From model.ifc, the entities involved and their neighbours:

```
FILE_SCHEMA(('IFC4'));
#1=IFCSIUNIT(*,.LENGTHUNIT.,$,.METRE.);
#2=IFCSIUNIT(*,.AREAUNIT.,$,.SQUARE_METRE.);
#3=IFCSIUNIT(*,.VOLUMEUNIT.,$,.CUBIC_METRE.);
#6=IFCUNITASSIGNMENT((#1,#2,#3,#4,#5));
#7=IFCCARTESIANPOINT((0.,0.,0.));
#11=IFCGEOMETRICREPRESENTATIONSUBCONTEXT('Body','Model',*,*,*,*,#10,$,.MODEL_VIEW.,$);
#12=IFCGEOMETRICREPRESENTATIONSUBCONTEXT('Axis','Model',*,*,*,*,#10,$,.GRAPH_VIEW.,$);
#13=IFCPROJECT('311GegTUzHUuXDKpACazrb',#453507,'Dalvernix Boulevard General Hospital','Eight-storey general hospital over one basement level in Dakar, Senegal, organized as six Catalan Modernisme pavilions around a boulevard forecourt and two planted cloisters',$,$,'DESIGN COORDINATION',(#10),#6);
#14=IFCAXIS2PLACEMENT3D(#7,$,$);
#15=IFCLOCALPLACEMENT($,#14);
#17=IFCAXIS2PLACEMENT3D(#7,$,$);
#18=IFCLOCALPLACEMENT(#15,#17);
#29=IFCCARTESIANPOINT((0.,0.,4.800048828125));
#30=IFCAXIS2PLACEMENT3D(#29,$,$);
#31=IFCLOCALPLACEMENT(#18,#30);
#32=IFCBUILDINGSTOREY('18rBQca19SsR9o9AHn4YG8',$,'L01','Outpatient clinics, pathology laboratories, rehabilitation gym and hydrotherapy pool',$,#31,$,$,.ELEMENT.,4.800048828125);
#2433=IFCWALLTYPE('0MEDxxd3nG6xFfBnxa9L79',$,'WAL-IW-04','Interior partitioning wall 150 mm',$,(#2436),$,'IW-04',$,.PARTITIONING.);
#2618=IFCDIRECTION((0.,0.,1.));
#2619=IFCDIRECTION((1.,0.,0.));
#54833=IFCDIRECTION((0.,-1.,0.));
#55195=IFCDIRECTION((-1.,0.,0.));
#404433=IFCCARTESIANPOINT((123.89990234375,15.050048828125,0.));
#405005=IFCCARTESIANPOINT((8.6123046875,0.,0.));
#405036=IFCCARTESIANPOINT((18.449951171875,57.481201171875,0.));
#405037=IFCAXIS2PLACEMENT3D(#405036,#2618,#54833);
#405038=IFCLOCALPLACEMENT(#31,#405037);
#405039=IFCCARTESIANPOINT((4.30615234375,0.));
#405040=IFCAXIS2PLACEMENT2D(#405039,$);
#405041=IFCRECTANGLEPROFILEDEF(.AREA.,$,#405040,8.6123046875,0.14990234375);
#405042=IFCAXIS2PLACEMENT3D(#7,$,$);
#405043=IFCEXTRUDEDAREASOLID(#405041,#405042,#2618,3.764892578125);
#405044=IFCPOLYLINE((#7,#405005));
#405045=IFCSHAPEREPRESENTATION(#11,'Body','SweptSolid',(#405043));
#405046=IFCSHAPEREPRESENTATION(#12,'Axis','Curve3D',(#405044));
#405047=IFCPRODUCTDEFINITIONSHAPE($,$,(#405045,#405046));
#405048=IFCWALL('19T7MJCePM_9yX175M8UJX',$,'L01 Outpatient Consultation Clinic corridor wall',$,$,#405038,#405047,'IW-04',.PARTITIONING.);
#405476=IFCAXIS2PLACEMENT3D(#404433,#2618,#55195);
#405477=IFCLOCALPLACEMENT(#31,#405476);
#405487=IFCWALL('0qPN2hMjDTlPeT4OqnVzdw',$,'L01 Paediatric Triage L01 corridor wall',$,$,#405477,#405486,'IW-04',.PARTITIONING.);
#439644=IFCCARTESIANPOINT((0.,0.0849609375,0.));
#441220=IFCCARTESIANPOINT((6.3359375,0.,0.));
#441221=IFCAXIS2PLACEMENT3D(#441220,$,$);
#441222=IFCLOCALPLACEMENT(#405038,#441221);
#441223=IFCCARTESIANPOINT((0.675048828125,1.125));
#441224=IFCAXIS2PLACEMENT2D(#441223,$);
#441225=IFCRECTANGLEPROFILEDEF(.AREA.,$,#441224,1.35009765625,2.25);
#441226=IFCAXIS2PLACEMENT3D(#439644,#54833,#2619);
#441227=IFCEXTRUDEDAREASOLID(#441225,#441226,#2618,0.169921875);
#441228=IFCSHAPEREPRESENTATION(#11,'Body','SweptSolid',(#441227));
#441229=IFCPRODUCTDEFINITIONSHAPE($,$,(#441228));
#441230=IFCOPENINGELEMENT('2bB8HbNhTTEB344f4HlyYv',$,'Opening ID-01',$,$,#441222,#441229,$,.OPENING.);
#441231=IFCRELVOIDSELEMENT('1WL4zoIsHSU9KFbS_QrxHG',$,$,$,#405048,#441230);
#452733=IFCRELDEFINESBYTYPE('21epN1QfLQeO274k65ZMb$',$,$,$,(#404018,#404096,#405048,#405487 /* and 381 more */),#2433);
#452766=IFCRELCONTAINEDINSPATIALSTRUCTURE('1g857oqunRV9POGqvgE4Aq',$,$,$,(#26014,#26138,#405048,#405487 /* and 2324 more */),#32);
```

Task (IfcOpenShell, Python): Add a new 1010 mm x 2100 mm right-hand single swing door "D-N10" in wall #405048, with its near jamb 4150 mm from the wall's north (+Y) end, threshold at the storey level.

```python
import numpy as np
import ifcopenshell
import ifcopenshell.api.feature
import ifcopenshell.api.geometry
import ifcopenshell.api.root
import ifcopenshell.api.spatial
import ifcopenshell.geom
import ifcopenshell.util.element
import ifcopenshell.util.placement
import ifcopenshell.util.representation
import ifcopenshell.util.shape
import ifcopenshell.util.unit

model = ifcopenshell.open("model.ifc")
unit_scale = ifcopenshell.util.unit.calculate_unit_scale(model)
settings = ifcopenshell.geom.settings()


def volume(element):
    """Net volume in cubic metres, openings subtracted."""
    shape = ifcopenshell.geom.create_shape(settings, element)
    return ifcopenshell.util.shape.get_volume(shape.geometry)


wall = model.by_id(405048)
storey = ifcopenshell.util.element.get_container(wall, ifc_class="IfcBuildingStorey")
context = ifcopenshell.util.representation.get_context(model, "Model", "Body", "MODEL_VIEW")
before = volume(wall)

width, height, from_end, sill = 1.01, 2.1, 4.15, 0.0  # metres

# The wall runs along its own X axis, and the end named is its -X end.
wall_shape = ifcopenshell.geom.create_shape(settings, wall)
x, y, z = ifcopenshell.util.shape.get_vertices(wall_shape.geometry).T
start = x.min() + from_end
face, thickness = float(y.min()), float(y.max() - y.min())
wall_matrix = ifcopenshell.util.placement.get_local_placement(wall.ObjectPlacement)
level = ifcopenshell.util.placement.get_local_placement(storey.ObjectPlacement)[2, 3]


def in_wall(x, y):
    """Placement at x, y metres in the wall's axes, at sill height."""
    matrix = wall_matrix.copy()
    matrix[:, 3] = wall_matrix @ np.array([x / unit_scale, y / unit_scale, 0.0, 1.0])
    matrix[2, 3] = level + sill / unit_scale
    return matrix


# Opening: a box that overshoots both wall faces by 50 mm.
opening = ifcopenshell.api.root.create_entity(model, ifc_class="IfcOpeningElement", predefined_type="OPENING")
box = ifcopenshell.api.geometry.add_wall_representation(
    model, context=context, length=width, height=height, thickness=thickness + 0.1
)
ifcopenshell.api.geometry.assign_representation(model, product=opening, representation=box)
ifcopenshell.api.geometry.edit_object_placement(model, product=opening, matrix=in_wall(start, face - 0.05), is_si=False)
ifcopenshell.api.feature.add_feature(model, feature=opening, element=wall)

door = ifcopenshell.api.root.create_entity(model, ifc_class="IfcDoor", name="D-N10", predefined_type="DOOR")
door.OverallWidth, door.OverallHeight = width / unit_scale, height / unit_scale
door.OperationType = "SINGLE_SWING_RIGHT"
body = ifcopenshell.api.geometry.add_door_representation(
    model,
    context=context,
    overall_width=door.OverallWidth,
    overall_height=door.OverallHeight,
    operation_type="SINGLE_SWING_RIGHT",
    lining_properties={"LiningDepth": thickness / unit_scale, "ThresholdDepth": thickness / unit_scale},
)
ifcopenshell.api.geometry.assign_representation(model, product=door, representation=body)
ifcopenshell.api.spatial.assign_container(model, products=[door], relating_structure=storey)
ifcopenshell.api.feature.add_filling(model, opening=opening, element=door)

# The lining spans the wall, so the door starts at the wall face.
ifcopenshell.api.geometry.edit_object_placement(model, product=door, matrix=in_wall(start, face), is_si=False)

after = volume(wall)

print(f"wall volume {before:.3f} -> {after:.3f} m3")

model.write("model_v2.ifc")
```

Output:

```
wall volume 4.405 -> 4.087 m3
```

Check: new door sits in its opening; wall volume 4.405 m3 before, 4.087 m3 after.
